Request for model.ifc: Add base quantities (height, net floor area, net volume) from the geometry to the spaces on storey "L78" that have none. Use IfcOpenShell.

First a look at what the model holds.

```python
import ifcopenshell
import ifcopenshell.util.element
import ifcopenshell.util.unit

model = ifcopenshell.open("model.ifc")
print(model.schema)
for unit_type in ("LENGTHUNIT", "AREAUNIT", "VOLUMEUNIT"):
    print(unit_type, ifcopenshell.util.unit.calculate_unit_scale(model, unit_type))
storey = next(s for s in model.by_type("IfcBuildingStorey") if s.Name == "L78")
spaces = [e for e in ifcopenshell.util.element.get_decomposition(storey) if e.is_a("IfcSpace")]
for e in sorted(spaces, key=lambda e: e.id()):
    print(e.id(), e.is_a(), e.Name, list(ifcopenshell.util.element.get_psets(e, qtos_only=True)), sep=" | ")
```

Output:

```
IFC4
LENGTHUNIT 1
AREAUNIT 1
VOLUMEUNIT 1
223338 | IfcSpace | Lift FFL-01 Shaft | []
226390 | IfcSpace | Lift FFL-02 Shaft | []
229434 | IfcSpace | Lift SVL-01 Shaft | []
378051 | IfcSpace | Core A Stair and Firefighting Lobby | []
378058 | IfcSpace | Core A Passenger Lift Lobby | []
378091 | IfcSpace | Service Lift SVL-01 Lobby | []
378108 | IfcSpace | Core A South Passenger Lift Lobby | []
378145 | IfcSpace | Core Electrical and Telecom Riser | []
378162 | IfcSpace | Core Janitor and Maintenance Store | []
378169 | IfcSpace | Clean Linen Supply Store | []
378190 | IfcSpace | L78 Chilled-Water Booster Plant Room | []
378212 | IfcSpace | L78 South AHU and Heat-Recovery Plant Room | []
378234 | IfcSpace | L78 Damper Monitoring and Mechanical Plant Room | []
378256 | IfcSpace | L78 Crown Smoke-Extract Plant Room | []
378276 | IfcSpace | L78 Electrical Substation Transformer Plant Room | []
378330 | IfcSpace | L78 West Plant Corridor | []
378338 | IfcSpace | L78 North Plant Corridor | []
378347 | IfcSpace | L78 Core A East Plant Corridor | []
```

```python
import ifcopenshell
import ifcopenshell.api.pset
import ifcopenshell.geom
import ifcopenshell.util.element
import ifcopenshell.util.shape
import ifcopenshell.util.unit

model = ifcopenshell.open("model.ifc")
unit_scale = ifcopenshell.util.unit.calculate_unit_scale(model)
area_scale = ifcopenshell.util.unit.calculate_unit_scale(model, "AREAUNIT")
volume_scale = ifcopenshell.util.unit.calculate_unit_scale(model, "VOLUMEUNIT")
settings = ifcopenshell.geom.settings()

storey = next(s for s in model.by_type("IfcBuildingStorey") if s.Name == "L78")
spaces = [e for e in ifcopenshell.util.element.get_decomposition(storey) if e.is_a("IfcSpace")]

for e in sorted(spaces, key=lambda e: e.id()):
    if ifcopenshell.util.element.get_psets(e, qtos_only=True, should_inherit=False):
        continue
    # Geometry comes back in metres, in the element's own axes.
    shape = ifcopenshell.geom.create_shape(settings, e)
    values = {
        "Height": ifcopenshell.util.shape.get_z(shape.geometry) / unit_scale,
        "NetFloorArea": ifcopenshell.util.shape.get_footprint_area(shape.geometry) / area_scale,
        "NetVolume": ifcopenshell.util.shape.get_volume(shape.geometry) / volume_scale,
    }
    qto = ifcopenshell.api.pset.add_qto(model, product=e, name="Qto_SpaceBaseQuantities")
    ifcopenshell.api.pset.edit_qto(model, qto=qto, properties=values)
    print(e.id(), {k: round(v, 3) for k, v in values.items()})

model.write("model_updated.ifc")
```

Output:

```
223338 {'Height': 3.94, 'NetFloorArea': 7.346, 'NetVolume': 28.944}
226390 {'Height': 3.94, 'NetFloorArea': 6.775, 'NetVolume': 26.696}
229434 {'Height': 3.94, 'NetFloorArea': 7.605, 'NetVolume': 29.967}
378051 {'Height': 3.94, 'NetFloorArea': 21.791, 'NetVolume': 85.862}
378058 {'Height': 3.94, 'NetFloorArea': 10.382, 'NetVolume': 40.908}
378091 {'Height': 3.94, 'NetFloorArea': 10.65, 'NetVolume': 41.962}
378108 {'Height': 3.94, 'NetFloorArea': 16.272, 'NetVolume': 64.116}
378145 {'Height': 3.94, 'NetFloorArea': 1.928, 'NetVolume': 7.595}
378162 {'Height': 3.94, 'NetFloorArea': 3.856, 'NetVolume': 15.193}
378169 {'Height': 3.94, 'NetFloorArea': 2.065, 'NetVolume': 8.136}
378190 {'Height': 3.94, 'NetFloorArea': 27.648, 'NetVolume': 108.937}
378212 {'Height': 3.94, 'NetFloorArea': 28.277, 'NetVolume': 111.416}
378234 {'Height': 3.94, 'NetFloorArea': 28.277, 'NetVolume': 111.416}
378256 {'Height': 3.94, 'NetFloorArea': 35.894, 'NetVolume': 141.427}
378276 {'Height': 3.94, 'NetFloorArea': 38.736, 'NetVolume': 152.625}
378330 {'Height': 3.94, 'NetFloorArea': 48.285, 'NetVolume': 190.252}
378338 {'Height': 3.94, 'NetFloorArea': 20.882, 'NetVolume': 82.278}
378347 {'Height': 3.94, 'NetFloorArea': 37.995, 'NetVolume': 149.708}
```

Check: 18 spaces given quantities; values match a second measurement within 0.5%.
